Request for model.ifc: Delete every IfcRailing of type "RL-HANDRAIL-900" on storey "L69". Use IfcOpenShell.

First a look at what the model holds.

```python
import ifcopenshell
import ifcopenshell.util.element

model = ifcopenshell.open("model.ifc")
print(model.schema)
storey = next(s for s in model.by_type("IfcBuildingStorey") if s.Name == "L69")
railings = [e for e in ifcopenshell.util.element.get_decomposition(storey) if e.is_a("IfcRailing")]
seen = {}
for e in railings:
    element_type = ifcopenshell.util.element.get_type(e)
    name = element_type.Name if element_type not in (None, e) else None
    seen[name] = seen.get(name, 0) + 1
for name, count in sorted(seen.items(), key=str):
    print(count, "x", name)
```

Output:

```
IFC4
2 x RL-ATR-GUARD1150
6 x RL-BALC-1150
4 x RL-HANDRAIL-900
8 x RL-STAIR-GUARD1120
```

```python
import ifcopenshell
import ifcopenshell.api.root
import ifcopenshell.util.element

model = ifcopenshell.open("model.ifc")

storey = next(s for s in model.by_type("IfcBuildingStorey") if s.Name == "L69")
railings = [e for e in ifcopenshell.util.element.get_decomposition(storey) if e.is_a("IfcRailing")]
targets = [e for e in railings if (t := ifcopenshell.util.element.get_type(e)) not in (None, e) and t.Name == "RL-HANDRAIL-900"]

for e in targets:
    ifcopenshell.api.root.remove_product(model, product=e)
print(len(targets), "removed")

model.write("model-out.ifc")
```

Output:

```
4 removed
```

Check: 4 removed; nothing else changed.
